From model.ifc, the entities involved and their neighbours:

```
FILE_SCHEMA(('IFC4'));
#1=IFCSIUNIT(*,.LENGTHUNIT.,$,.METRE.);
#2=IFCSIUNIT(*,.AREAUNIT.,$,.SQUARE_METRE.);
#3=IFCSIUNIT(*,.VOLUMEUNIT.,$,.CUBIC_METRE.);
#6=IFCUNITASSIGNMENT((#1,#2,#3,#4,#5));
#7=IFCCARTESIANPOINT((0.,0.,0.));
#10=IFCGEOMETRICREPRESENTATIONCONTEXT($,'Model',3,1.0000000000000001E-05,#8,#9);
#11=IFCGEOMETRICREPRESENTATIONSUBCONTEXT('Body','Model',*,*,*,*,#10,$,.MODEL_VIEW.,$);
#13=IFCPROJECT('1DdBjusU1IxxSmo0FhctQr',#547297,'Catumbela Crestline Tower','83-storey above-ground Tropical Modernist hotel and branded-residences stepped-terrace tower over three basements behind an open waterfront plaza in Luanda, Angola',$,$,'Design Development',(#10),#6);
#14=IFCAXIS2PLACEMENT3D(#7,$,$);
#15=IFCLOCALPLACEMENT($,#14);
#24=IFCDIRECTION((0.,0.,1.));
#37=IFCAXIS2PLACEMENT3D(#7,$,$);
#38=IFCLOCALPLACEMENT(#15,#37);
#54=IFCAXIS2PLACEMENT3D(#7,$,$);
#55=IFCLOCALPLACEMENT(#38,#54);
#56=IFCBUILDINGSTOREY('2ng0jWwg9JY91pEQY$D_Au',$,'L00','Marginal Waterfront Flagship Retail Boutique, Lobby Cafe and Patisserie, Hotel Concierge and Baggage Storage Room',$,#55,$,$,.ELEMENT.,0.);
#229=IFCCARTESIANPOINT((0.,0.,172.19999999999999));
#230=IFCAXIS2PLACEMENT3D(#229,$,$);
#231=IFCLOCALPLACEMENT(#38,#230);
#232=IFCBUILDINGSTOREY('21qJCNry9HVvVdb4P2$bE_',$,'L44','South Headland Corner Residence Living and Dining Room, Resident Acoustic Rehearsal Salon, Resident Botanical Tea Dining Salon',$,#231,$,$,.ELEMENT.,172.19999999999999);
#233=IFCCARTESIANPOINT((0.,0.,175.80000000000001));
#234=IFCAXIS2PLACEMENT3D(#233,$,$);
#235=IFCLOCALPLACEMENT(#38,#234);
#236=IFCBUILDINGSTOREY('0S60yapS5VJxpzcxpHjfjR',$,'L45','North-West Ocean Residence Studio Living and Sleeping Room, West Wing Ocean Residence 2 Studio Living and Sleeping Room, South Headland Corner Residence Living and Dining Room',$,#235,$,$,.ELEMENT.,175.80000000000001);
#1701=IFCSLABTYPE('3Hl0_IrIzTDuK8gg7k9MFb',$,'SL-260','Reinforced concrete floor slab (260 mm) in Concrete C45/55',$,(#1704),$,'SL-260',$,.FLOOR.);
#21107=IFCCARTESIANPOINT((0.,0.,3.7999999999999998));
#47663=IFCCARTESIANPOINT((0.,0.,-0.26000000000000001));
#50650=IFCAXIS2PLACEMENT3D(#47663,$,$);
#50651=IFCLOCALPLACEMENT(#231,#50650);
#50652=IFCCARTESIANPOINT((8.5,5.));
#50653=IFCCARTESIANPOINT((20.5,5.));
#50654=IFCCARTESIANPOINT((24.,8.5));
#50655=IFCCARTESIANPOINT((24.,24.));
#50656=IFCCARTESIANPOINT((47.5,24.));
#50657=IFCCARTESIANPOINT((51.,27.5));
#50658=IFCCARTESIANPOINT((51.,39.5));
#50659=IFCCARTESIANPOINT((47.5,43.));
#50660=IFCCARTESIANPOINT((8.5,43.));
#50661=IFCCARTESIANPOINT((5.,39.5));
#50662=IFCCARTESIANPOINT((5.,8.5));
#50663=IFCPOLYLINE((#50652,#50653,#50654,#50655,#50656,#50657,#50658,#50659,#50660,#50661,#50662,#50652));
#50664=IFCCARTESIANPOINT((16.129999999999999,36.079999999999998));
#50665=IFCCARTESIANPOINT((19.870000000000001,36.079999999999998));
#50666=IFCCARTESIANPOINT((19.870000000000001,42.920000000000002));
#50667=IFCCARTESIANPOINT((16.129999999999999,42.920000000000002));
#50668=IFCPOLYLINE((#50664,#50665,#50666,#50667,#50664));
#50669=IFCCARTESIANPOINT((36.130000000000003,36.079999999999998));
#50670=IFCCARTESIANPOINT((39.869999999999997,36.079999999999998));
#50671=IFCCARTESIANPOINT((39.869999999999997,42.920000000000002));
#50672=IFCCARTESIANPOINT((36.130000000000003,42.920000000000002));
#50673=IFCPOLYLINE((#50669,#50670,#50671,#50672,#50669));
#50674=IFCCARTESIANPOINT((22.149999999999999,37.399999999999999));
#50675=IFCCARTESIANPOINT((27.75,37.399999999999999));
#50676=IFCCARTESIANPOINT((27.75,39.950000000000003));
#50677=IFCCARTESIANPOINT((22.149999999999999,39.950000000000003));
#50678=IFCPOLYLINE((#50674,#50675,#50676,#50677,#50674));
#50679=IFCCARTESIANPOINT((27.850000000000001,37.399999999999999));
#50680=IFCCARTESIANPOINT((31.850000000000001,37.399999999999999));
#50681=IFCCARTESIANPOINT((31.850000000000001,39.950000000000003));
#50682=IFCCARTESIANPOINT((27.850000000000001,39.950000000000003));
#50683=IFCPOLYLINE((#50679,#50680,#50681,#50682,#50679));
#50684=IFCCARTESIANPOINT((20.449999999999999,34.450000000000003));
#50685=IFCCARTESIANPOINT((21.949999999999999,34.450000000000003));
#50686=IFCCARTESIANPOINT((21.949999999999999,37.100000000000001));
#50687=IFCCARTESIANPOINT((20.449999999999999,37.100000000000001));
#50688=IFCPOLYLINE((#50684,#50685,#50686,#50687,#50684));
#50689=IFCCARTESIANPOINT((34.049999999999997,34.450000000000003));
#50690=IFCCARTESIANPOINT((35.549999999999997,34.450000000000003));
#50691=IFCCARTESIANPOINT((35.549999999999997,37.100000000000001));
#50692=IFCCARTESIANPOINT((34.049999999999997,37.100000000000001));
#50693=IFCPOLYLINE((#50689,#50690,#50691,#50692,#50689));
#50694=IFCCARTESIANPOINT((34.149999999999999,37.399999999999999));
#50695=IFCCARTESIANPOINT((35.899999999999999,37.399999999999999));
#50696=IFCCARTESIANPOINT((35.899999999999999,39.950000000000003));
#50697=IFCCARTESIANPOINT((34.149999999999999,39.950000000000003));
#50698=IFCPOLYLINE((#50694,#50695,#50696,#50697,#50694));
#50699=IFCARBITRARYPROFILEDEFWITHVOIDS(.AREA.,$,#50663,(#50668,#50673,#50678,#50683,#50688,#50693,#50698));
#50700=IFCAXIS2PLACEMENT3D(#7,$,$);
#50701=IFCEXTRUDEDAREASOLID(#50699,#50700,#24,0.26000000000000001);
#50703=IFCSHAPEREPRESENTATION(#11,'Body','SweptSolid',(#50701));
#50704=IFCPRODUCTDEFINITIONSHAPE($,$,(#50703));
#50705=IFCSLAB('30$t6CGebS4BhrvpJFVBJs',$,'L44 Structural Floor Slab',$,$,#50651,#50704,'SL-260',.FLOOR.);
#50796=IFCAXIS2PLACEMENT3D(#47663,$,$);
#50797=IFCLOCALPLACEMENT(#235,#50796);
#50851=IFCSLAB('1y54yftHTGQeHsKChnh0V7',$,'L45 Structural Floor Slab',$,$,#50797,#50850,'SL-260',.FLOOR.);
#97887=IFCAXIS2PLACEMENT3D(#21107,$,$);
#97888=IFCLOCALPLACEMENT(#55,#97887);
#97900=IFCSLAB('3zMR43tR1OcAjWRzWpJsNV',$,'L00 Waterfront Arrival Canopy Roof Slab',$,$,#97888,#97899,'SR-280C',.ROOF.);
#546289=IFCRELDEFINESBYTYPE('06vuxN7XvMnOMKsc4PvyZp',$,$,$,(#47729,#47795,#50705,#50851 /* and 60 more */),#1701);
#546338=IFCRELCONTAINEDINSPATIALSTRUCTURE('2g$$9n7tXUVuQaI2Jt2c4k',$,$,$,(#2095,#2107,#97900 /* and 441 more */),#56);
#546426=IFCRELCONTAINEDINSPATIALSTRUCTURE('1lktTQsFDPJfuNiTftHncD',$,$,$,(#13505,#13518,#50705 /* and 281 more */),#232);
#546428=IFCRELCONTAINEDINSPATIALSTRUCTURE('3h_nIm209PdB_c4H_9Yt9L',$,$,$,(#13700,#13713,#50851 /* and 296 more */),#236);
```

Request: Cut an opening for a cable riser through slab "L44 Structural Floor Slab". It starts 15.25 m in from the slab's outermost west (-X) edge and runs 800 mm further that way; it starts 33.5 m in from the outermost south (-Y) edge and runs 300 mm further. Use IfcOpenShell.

```python
import numpy as np
import ifcopenshell
import ifcopenshell.api.feature
import ifcopenshell.api.geometry
import ifcopenshell.api.root
import ifcopenshell.geom
import ifcopenshell.util.placement
import ifcopenshell.util.representation
import ifcopenshell.util.shape
import ifcopenshell.util.unit

model = ifcopenshell.open("model.ifc")
unit_scale = ifcopenshell.util.unit.calculate_unit_scale(model)
settings = ifcopenshell.geom.settings()


def volume(element):
    """Net volume in cubic metres, openings subtracted."""
    shape = ifcopenshell.geom.create_shape(settings, element)
    return ifcopenshell.util.shape.get_volume(shape.geometry)


slab = model.by_guid("30$t6CGebS4BhrvpJFVBJs")
before = volume(slab)

# Extent in the slab's own axes, in metres. The edges named are its -X and -Y sides.
slab_shape = ifcopenshell.geom.create_shape(settings, slab)
vertices = ifcopenshell.util.shape.get_vertices(slab_shape.geometry)
x_min, y_min, bottom = vertices.min(axis=0)
top = vertices[:, 2].max()

opening = ifcopenshell.api.root.create_entity(model, ifc_class="IfcOpeningElement", name="Cable riser opening", predefined_type="OPENING")
context = ifcopenshell.util.representation.get_context(model, "Model", "Body", "MODEL_VIEW")
width, depth = 0.8, 0.3
outline = [(0.0, 0.0), (width, 0.0), (width, depth), (0.0, depth), (0.0, 0.0)]
# Overshoot both faces by 50 mm so the cut is clean.
shape = ifcopenshell.api.geometry.add_slab_representation(
    model, context=context, depth=top - bottom + 0.1, polyline=outline
)
ifcopenshell.api.geometry.assign_representation(model, product=opening, representation=shape)

matrix = ifcopenshell.util.placement.get_local_placement(slab.ObjectPlacement)
matrix[:, 3] = matrix @ np.append(np.array([x_min + 15.25, y_min + 33.5, bottom - 0.05]) / unit_scale, 1.0)
ifcopenshell.api.geometry.edit_object_placement(model, product=opening, matrix=matrix, is_si=False)
ifcopenshell.api.feature.add_feature(model, feature=opening, element=slab)

after = volume(slab)

print(f"slab volume {before:.3f} -> {after:.3f} m3")

model.write("model_updated.ifc")
```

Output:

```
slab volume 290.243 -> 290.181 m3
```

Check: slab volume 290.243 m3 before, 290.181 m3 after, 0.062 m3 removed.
